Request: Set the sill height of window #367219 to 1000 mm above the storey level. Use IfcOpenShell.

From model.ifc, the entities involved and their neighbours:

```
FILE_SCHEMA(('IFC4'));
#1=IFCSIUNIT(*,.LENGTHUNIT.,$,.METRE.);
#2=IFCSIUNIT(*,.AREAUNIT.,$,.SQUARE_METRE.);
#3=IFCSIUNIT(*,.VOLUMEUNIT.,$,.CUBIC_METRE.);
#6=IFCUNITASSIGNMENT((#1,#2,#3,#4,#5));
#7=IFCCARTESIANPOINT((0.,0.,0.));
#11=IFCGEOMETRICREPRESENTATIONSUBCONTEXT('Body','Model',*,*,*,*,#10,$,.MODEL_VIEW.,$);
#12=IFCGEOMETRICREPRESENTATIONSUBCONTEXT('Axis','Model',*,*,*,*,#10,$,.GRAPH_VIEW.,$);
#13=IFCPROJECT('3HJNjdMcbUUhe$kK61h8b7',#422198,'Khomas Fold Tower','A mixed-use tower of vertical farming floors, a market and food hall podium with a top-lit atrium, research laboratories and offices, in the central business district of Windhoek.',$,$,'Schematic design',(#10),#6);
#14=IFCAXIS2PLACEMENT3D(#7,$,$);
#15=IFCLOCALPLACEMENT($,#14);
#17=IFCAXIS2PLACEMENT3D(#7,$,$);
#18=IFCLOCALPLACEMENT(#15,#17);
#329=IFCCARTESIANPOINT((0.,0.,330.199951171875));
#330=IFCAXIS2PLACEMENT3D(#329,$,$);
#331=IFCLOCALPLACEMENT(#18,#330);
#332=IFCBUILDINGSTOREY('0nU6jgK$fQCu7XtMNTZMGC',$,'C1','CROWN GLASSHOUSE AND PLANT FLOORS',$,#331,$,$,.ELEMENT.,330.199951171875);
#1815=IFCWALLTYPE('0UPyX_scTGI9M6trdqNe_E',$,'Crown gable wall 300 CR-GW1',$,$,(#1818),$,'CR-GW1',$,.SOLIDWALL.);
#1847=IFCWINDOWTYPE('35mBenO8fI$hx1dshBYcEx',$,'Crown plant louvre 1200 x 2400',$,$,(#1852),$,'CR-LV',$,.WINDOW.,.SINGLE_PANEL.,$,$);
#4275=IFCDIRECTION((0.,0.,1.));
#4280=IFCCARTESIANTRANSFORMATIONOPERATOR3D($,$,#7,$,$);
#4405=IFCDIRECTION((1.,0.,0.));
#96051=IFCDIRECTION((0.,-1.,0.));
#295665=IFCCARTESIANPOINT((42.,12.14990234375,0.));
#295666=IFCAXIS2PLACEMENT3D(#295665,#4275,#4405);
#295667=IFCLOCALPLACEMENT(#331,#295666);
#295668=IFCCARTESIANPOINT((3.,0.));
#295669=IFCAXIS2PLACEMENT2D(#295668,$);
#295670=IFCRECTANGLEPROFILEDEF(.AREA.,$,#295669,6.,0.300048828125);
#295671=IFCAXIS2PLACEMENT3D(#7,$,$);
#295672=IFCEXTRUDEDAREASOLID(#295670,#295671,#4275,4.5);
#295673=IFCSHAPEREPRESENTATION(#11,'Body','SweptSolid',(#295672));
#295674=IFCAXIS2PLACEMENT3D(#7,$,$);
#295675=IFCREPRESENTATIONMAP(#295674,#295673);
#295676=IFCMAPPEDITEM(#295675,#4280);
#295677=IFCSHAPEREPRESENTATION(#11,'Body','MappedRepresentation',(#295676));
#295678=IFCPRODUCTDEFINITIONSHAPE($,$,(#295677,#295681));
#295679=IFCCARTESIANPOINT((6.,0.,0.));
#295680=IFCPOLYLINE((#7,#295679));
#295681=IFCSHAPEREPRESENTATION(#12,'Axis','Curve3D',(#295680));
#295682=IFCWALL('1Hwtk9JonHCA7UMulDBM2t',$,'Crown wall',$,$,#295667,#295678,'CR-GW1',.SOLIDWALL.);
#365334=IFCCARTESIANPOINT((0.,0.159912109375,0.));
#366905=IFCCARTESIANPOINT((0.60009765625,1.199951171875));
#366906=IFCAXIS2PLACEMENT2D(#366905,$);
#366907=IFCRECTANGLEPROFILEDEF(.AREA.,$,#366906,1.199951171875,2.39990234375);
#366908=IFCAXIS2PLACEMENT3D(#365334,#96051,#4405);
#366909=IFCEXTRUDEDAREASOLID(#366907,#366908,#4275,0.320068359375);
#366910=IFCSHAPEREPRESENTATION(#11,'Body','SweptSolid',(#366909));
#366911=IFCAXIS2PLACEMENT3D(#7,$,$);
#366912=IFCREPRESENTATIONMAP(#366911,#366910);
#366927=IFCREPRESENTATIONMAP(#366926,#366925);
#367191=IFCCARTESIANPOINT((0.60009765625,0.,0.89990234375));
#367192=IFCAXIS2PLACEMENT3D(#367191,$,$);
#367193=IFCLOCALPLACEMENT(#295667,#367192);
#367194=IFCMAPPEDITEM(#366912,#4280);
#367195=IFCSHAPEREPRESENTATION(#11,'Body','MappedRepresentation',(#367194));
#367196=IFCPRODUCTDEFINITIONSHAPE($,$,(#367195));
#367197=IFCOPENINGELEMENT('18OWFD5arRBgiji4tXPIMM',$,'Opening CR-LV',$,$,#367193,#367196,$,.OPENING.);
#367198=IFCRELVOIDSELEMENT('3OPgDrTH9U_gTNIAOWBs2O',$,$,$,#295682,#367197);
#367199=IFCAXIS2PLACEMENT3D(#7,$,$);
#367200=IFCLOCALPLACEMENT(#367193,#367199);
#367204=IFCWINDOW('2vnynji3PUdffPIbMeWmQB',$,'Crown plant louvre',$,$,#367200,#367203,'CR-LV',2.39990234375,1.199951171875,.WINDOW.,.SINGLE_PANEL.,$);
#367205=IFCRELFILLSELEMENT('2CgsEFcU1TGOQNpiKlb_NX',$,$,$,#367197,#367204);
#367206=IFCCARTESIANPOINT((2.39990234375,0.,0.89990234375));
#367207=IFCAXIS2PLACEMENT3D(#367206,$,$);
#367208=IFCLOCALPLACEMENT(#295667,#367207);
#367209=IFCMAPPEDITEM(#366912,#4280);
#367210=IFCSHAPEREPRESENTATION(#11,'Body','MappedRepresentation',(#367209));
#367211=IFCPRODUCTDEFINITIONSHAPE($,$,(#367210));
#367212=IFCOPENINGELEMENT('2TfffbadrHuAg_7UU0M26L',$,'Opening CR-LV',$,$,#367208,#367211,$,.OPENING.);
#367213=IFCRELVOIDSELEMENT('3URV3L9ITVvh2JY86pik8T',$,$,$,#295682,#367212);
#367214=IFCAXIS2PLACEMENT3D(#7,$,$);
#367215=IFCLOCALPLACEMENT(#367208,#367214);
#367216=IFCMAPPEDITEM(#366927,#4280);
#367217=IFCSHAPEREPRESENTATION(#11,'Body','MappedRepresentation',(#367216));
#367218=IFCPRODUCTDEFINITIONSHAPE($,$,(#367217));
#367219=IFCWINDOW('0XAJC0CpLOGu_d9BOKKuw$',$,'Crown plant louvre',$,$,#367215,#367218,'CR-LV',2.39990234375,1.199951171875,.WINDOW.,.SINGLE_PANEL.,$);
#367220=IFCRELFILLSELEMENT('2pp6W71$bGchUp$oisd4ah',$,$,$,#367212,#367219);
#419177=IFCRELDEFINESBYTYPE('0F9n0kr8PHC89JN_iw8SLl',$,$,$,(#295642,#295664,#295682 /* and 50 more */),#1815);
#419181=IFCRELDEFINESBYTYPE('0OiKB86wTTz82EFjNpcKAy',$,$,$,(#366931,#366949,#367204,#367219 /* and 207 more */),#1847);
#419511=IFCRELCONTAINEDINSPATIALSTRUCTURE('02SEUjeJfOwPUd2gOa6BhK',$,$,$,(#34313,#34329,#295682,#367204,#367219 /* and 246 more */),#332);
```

```python
import numpy as np
import ifcopenshell
import ifcopenshell.api.geometry
import ifcopenshell.geom
import ifcopenshell.util.element
import ifcopenshell.util.placement
import ifcopenshell.util.shape
import ifcopenshell.util.unit

model = ifcopenshell.open("model.ifc")
unit_scale = ifcopenshell.util.unit.calculate_unit_scale(model)

window = model.by_guid("0XAJC0CpLOGu_d9BOKKuw$")
opening = window.FillsVoids[0].RelatingOpeningElement
storey = ifcopenshell.util.element.get_container(window, ifc_class="IfcBuildingStorey")
level = ifcopenshell.util.placement.get_local_placement(storey.ObjectPlacement)[2, 3]

# The opening's origin need not be at the sill, so measure its lowest point.
shape = ifcopenshell.geom.create_shape(ifcopenshell.geom.settings(), opening)
bottom = ifcopenshell.util.shape.get_shape_bottom_elevation(shape, shape.geometry) / unit_scale
dz = level + 1 / unit_scale - bottom

shift = np.array([0.0, 0.0, dz])
# The window is placed relative to its opening, so it follows when the opening moves.
matrix = ifcopenshell.util.placement.get_local_placement(opening.ObjectPlacement)
matrix[:3, 3] += shift
ifcopenshell.api.geometry.edit_object_placement(
    model, product=opening, matrix=matrix, is_si=False, should_transform_children=True
)

print(f"moved by {dz * unit_scale:+.3f} m")

model.write("model_updated.ifc")
```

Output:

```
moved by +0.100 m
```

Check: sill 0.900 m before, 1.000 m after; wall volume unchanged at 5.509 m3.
